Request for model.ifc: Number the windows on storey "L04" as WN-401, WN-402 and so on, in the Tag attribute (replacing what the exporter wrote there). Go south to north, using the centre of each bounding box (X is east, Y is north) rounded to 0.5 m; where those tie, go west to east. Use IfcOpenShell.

First a look at what the model holds.

```python
import ifcopenshell
import ifcopenshell.util.element
import ifcopenshell.util.placement

model = ifcopenshell.open("model.ifc")
print(model.schema)
storey = next(s for s in model.by_type("IfcBuildingStorey") if s.Name == "L04")
windows = [e for e in ifcopenshell.util.element.get_decomposition(storey) if e.is_a("IfcWindow")]
for e in sorted(windows, key=lambda e: e.id()):
    origin = ifcopenshell.util.placement.get_local_placement(e.ObjectPlacement)[:3, 3]
    print(e.id(), e.Tag, e.Name, origin.round(2) + 0.0, sep=" | ")
```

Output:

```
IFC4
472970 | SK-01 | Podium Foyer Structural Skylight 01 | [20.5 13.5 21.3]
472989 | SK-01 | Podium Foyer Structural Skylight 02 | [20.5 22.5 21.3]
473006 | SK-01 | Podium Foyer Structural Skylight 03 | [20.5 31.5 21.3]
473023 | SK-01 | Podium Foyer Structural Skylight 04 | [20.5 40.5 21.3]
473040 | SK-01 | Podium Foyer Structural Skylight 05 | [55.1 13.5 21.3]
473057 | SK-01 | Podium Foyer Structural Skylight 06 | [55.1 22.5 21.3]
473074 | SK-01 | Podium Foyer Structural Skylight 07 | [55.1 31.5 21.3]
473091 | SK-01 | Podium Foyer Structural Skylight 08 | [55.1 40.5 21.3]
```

```python
import ifcopenshell
import ifcopenshell.geom
import ifcopenshell.util.element
import ifcopenshell.util.shape

model = ifcopenshell.open("model.ifc")
settings = ifcopenshell.geom.settings()
settings.set("use-world-coords", True)


def centre(element):
    shape = ifcopenshell.geom.create_shape(settings, element)
    return ifcopenshell.util.shape.get_bbox_centroid(shape.geometry)


storey = next(s for s in model.by_type("IfcBuildingStorey") if s.Name == "L04")
windows = [e for e in ifcopenshell.util.element.get_decomposition(storey) if e.is_a("IfcWindow")]

# Insertion points can sit at a corner or the storey origin, so sort by the geometry (in metres).
centres = {e: centre(e) for e in windows}
windows.sort(key=lambda e: (round(centres[e][1] / 0.5), centres[e][0]))

for i, e in enumerate(windows, start=1):
    number = f"WN-4{i:02d}"
    e.Tag = number
    print(e.id(), number)

model.write("model_edited.ifc")
```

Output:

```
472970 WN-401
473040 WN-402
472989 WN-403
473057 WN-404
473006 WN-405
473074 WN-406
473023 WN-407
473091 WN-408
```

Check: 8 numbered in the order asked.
